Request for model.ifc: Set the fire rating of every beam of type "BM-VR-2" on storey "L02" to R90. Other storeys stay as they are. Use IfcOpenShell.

First a look at what the model holds.

```python
import ifcopenshell
import ifcopenshell.util.element

model = ifcopenshell.open("model.ifc")
print(model.schema)
storey = next(s for s in model.by_type("IfcBuildingStorey") if s.Name == "L02")
beams = [e for e in ifcopenshell.util.element.get_decomposition(storey) if e.is_a("IfcBeam")]
seen = {}
for e in beams:
    element_type = ifcopenshell.util.element.get_type(e)
    key = (element_type.Name if element_type != e and element_type else None, ifcopenshell.util.element.get_pset(e, "Pset_BeamCommon", "FireRating"))
    seen[key] = seen.get(key, 0) + 1
for (name, value), count in sorted(seen.items(), key=str):
    print(count, "x", name, "|", value)
```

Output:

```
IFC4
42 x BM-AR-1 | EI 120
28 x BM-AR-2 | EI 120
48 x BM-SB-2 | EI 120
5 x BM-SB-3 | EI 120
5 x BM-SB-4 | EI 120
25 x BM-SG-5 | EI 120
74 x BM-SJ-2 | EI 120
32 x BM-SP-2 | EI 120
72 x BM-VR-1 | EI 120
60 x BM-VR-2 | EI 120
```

```python
import ifcopenshell
import ifcopenshell.api.pset
import ifcopenshell.util.element

model = ifcopenshell.open("model.ifc")

storey = next(s for s in model.by_type("IfcBuildingStorey") if s.Name == "L02")
beams = [e for e in ifcopenshell.util.element.get_decomposition(storey) if e.is_a("IfcBeam")]

count = 0
for e in beams:
    element_type = ifcopenshell.util.element.get_type(e)
    if element_type in (None, e) or element_type.Name != "BM-VR-2":
        continue
    # add_pset returns the element's existing set when there is one.
    pset = ifcopenshell.api.pset.add_pset(model, product=e, name="Pset_BeamCommon")
    ifcopenshell.api.pset.edit_pset(model, pset=pset, properties={"FireRating": "R90"})
    count += 1

print(count, "beams updated")

model.write("model_v2.ifc")
```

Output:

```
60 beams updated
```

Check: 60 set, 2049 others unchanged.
